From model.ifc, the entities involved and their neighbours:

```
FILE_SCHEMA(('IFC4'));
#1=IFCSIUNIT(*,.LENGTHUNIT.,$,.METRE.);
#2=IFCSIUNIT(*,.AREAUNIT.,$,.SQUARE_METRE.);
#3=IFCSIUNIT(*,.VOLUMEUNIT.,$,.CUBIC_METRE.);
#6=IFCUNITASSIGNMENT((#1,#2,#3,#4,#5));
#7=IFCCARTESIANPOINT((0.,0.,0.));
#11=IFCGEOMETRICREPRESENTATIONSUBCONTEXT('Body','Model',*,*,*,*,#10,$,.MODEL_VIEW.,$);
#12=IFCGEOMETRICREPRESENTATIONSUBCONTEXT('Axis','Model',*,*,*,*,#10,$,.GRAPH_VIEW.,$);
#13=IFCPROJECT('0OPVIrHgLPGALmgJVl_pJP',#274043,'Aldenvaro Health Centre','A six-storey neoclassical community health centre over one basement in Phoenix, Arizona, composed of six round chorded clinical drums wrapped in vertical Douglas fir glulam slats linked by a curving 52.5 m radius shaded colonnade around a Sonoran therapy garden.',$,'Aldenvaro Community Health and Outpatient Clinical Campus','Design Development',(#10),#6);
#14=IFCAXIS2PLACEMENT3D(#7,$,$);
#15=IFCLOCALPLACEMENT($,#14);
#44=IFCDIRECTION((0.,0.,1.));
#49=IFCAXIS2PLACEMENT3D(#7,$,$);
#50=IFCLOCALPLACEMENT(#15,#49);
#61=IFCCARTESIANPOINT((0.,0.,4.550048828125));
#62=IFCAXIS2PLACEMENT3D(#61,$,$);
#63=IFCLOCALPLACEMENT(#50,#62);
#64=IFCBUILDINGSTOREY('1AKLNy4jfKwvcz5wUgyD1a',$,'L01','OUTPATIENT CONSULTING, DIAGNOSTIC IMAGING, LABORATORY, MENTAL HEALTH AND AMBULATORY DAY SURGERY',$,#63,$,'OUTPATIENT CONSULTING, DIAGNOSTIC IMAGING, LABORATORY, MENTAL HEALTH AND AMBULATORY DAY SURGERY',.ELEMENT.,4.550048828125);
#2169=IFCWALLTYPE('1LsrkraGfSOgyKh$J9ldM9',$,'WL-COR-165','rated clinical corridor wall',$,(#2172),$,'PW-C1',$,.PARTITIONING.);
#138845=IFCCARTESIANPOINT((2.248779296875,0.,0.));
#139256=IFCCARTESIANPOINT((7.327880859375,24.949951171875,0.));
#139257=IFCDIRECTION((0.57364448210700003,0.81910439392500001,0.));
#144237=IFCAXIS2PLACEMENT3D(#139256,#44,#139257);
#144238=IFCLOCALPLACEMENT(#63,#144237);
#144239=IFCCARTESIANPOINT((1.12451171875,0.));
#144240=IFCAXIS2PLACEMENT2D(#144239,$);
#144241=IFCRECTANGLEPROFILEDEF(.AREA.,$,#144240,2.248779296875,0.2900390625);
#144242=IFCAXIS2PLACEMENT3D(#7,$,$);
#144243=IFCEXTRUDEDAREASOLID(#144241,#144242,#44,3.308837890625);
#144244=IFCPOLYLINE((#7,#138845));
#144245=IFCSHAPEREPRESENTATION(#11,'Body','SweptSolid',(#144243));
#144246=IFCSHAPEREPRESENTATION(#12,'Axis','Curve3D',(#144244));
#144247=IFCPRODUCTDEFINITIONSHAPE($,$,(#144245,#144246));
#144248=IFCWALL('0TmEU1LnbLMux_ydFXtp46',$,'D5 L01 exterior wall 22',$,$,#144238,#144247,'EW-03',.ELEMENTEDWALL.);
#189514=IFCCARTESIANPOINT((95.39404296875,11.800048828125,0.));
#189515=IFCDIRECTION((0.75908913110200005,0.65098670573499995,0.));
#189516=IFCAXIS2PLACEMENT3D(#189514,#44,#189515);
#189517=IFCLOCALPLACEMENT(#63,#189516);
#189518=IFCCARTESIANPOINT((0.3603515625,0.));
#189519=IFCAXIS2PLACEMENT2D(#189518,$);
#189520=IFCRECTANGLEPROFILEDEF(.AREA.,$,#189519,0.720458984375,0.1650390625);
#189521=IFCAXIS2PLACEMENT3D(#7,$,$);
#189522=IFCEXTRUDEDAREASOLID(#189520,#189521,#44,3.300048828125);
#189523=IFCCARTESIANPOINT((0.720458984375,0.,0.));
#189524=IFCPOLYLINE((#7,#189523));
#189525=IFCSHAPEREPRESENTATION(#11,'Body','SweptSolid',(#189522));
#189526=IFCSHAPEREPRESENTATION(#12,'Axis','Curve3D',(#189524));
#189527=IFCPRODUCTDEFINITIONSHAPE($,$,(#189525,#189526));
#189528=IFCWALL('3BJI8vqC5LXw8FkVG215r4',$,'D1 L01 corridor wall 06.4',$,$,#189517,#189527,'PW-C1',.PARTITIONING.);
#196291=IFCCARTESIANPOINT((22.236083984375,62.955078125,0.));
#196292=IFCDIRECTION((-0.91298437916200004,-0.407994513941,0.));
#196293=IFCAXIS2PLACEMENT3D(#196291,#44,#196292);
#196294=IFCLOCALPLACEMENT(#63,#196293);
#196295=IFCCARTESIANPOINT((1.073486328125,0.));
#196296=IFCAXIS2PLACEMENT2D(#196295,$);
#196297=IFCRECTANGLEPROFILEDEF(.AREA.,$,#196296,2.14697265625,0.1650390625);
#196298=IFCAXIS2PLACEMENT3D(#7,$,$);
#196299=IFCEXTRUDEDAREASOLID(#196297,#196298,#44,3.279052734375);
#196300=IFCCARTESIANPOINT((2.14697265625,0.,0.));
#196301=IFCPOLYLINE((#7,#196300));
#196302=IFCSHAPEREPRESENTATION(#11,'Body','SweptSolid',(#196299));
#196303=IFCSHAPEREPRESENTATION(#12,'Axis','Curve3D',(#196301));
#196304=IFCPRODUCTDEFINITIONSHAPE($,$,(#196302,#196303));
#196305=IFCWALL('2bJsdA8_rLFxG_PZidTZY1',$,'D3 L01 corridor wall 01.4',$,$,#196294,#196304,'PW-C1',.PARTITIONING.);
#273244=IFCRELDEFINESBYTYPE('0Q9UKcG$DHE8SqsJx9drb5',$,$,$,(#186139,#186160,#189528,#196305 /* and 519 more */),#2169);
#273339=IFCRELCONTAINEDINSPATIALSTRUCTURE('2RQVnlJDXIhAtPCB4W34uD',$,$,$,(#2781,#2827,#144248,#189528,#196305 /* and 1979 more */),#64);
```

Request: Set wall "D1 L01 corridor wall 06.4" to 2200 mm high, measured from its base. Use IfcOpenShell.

```python
import ifcopenshell
import ifcopenshell.geom
import ifcopenshell.util.representation
import ifcopenshell.util.shape

model = ifcopenshell.open("model.ifc")
settings = ifcopenshell.geom.settings()


def volume(element):
    """Net volume in cubic metres, openings subtracted."""
    shape = ifcopenshell.geom.create_shape(settings, element)
    return ifcopenshell.util.shape.get_volume(shape.geometry)


wall = model.by_guid("3BJI8vqC5LXw8FkVG215r4")
before = volume(wall)

body = ifcopenshell.util.representation.get_representation(wall, "Model", "Body")
solid = body.Items[0]
old_height = solid.Depth
solid.Depth = 2.2
after = volume(wall)

print(f"height {old_height:g} -> {solid.Depth:g}, volume {before:.3f} -> {after:.3f} m3")

model.write("model_rev.ifc")
```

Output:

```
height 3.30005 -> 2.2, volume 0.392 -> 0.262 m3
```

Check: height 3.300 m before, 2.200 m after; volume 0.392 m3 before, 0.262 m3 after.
